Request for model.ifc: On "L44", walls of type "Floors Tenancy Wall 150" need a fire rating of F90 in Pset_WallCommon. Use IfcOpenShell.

First a look at what the model holds.

```python
import ifcopenshell
import ifcopenshell.util.element

model = ifcopenshell.open("model.ifc")
print(model.schema)
storey = next(s for s in model.by_type("IfcBuildingStorey") if s.Name == "L44")
walls = [e for e in ifcopenshell.util.element.get_decomposition(storey) if e.is_a("IfcWall")]
seen = {}
for e in walls:
    element_type = ifcopenshell.util.element.get_type(e)
    key = (element_type.Name if element_type != e and element_type else None, ifcopenshell.util.element.get_pset(e, "Pset_WallCommon", "FireRating"))
    seen[key] = seen.get(key, 0) + 1
for (name, value), count in sorted(seen.items(), key=str):
    print(count, "x", name, "|", value)
```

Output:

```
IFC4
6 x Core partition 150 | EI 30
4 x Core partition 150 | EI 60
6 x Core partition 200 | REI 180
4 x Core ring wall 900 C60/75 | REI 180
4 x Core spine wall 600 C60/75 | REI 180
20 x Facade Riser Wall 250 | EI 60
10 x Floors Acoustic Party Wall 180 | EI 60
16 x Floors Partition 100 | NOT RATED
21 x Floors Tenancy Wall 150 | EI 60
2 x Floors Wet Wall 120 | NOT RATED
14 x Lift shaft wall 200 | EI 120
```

```python
import ifcopenshell
import ifcopenshell.api.pset
import ifcopenshell.util.element

model = ifcopenshell.open("model.ifc")

storey = next(s for s in model.by_type("IfcBuildingStorey") if s.Name == "L44")
walls = [e for e in ifcopenshell.util.element.get_decomposition(storey) if e.is_a("IfcWall")]

count = 0
for e in walls:
    element_type = ifcopenshell.util.element.get_type(e)
    if element_type in (None, e) or element_type.Name != "Floors Tenancy Wall 150":
        continue
    found = ifcopenshell.util.element.get_pset(e, "Pset_WallCommon", should_inherit=False)
    if found:
        pset = model.by_id(found["id"])
        if len(ifcopenshell.util.element.get_elements_by_pset(pset)) > 1:
            pset = ifcopenshell.api.pset.unshare_pset(model, products=[e], pset=pset)[0]
    else:
        pset = ifcopenshell.api.pset.add_pset(model, product=e, name="Pset_WallCommon")
    ifcopenshell.api.pset.edit_pset(model, pset=pset, properties={"FireRating": "F90"})
    count += 1

print(count, "walls updated")

model.write("model_updated.ifc")
```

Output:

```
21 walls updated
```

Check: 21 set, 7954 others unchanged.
